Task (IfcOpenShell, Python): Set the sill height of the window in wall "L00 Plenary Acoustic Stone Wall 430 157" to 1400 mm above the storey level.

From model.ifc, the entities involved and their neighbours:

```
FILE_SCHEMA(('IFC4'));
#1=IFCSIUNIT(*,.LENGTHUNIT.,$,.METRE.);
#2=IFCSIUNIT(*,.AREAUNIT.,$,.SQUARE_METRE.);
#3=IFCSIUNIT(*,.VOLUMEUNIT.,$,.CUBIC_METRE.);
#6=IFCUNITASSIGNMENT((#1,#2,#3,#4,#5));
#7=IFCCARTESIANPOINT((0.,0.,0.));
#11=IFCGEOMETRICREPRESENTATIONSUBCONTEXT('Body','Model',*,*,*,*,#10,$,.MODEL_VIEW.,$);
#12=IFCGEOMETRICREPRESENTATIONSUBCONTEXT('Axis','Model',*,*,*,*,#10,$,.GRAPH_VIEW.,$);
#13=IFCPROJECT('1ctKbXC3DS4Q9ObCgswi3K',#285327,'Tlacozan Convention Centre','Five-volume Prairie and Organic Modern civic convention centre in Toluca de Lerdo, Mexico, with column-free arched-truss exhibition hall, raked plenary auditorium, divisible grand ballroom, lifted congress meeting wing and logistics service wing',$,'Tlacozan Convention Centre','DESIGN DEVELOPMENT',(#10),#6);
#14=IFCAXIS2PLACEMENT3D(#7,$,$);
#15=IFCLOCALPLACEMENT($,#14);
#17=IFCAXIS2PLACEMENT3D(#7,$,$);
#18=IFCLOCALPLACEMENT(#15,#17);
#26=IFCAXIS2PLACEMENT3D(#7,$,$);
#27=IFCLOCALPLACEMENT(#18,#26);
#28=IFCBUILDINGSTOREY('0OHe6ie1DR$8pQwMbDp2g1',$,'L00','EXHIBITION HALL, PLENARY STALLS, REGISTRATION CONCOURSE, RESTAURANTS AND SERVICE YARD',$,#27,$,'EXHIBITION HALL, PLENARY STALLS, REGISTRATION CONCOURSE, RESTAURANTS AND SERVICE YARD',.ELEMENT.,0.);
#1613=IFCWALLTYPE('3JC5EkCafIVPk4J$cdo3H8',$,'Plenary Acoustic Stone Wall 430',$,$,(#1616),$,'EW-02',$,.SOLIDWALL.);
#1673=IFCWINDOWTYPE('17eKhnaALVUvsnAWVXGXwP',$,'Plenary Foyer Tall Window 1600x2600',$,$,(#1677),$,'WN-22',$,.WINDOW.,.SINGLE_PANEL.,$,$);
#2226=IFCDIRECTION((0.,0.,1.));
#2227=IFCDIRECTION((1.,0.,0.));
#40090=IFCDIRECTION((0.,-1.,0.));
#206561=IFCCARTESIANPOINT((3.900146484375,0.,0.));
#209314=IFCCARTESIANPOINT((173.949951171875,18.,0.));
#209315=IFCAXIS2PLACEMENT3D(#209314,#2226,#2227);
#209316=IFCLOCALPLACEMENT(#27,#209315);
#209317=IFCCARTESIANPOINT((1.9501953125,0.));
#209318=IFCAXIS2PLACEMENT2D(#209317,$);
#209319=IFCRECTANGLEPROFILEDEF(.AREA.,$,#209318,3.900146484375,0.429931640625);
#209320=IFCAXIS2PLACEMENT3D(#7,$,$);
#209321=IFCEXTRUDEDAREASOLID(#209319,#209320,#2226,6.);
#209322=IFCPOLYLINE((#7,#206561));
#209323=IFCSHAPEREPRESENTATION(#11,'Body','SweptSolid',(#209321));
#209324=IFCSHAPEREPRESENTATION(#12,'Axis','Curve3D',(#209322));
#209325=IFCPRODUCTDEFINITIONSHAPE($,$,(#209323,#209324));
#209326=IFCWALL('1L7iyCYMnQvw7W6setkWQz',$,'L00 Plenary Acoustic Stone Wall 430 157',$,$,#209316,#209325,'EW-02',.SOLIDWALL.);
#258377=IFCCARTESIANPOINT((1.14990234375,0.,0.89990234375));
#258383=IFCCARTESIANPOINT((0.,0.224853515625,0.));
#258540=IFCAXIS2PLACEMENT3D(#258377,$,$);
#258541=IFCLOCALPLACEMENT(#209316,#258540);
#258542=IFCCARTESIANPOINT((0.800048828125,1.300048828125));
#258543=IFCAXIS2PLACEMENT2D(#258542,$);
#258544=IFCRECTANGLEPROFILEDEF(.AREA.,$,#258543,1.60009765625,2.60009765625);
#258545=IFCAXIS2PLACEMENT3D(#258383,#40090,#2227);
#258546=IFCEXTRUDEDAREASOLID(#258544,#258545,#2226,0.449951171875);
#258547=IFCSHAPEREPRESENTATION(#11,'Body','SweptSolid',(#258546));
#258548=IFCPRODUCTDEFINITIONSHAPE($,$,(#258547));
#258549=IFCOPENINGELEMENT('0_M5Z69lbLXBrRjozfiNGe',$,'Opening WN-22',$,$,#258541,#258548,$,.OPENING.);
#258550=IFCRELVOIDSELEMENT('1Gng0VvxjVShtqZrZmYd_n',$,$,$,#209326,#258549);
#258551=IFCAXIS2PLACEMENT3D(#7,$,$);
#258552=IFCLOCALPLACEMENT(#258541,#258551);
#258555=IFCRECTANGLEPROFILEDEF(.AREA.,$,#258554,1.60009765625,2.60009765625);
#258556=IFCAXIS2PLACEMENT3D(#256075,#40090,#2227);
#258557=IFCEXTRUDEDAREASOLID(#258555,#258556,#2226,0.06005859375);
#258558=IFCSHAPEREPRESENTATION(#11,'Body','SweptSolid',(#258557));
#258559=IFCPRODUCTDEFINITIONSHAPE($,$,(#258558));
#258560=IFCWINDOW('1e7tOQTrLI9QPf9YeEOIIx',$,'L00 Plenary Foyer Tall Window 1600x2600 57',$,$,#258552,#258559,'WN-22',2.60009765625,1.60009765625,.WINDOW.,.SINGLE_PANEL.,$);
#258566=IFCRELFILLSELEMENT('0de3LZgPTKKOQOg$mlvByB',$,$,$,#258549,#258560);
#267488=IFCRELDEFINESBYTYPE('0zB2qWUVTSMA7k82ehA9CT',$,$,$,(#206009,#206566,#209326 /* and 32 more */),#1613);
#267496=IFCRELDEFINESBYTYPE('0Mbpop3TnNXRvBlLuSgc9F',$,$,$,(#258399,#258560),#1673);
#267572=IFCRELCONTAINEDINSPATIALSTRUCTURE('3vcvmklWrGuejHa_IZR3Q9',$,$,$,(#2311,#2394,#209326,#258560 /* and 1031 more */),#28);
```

```python
import numpy as np
import ifcopenshell
import ifcopenshell.api.geometry
import ifcopenshell.geom
import ifcopenshell.util.element
import ifcopenshell.util.placement
import ifcopenshell.util.shape
import ifcopenshell.util.unit

model = ifcopenshell.open("model.ifc")
unit_scale = ifcopenshell.util.unit.calculate_unit_scale(model)

window = model.by_id(258560)
opening = window.FillsVoids[0].RelatingOpeningElement
storey = ifcopenshell.util.element.get_container(window, ifc_class="IfcBuildingStorey")
level = ifcopenshell.util.placement.get_local_placement(storey.ObjectPlacement)[2, 3]

# The opening's origin need not be at the sill, so measure its lowest point.
shape = ifcopenshell.geom.create_shape(ifcopenshell.geom.settings(), opening)
bottom = ifcopenshell.util.shape.get_shape_bottom_elevation(shape, shape.geometry) / unit_scale
dz = level + 1.4 / unit_scale - bottom

shift = np.array([0.0, 0.0, dz])
# The window is placed relative to its opening, so it follows when the opening moves.
matrix = ifcopenshell.util.placement.get_local_placement(opening.ObjectPlacement)
matrix[:3, 3] += shift
ifcopenshell.api.geometry.edit_object_placement(
    model, product=opening, matrix=matrix, is_si=False, should_transform_children=True
)

print(f"moved by {dz * unit_scale:+.3f} m")

model.write("model_updated.ifc")
```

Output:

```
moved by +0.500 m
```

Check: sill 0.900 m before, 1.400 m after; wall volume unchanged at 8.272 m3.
